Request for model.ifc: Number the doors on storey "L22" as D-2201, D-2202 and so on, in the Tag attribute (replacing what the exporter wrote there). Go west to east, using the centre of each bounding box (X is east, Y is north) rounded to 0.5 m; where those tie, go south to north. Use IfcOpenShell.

First a look at what the model holds.

```python
import ifcopenshell
import ifcopenshell.util.element
import ifcopenshell.util.placement

model = ifcopenshell.open("model.ifc")
print(model.schema)
storey = next(s for s in model.by_type("IfcBuildingStorey") if s.Name == "L22")
doors = [e for e in ifcopenshell.util.element.get_decomposition(storey) if e.is_a("IfcDoor")]
for e in sorted(doors, key=lambda e: e.id()):
    origin = ifcopenshell.util.placement.get_local_placement(e.ObjectPlacement)[:3, 3]
    print(e.id(), e.Tag, e.Name, origin.round(2) + 0.0, sep=" | ")
```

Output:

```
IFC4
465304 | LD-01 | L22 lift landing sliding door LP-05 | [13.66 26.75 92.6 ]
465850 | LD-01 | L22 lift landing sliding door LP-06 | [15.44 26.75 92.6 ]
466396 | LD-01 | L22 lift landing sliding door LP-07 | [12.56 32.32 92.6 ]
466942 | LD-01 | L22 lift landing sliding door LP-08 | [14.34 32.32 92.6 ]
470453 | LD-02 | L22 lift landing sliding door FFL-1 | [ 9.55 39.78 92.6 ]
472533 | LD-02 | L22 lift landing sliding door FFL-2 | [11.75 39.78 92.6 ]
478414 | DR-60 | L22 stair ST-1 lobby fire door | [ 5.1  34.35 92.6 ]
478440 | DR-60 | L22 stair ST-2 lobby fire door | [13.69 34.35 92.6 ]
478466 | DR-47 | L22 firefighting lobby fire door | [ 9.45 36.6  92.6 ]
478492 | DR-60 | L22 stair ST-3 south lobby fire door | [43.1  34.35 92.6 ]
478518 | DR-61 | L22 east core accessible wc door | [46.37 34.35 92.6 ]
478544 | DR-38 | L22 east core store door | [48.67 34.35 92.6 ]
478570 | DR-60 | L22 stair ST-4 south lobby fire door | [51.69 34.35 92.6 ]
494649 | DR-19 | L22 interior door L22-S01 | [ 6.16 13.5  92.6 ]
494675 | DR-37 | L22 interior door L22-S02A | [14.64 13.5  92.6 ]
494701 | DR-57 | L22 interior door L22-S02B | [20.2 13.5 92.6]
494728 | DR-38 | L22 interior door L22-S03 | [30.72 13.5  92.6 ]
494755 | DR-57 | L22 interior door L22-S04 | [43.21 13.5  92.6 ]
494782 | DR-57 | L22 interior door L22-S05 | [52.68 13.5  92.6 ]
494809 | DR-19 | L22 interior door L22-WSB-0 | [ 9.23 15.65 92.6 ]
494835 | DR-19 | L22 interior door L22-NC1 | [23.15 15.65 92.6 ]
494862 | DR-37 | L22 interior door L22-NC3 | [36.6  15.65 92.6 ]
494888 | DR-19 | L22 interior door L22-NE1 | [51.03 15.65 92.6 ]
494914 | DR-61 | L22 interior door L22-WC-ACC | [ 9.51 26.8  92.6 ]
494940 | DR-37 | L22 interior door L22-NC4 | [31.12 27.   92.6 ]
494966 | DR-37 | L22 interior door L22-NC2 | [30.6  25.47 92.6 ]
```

```python
import ifcopenshell
import ifcopenshell.geom
import ifcopenshell.util.element
import ifcopenshell.util.shape

model = ifcopenshell.open("model.ifc")
settings = ifcopenshell.geom.settings()
settings.set("use-world-coords", True)


def centre(element):
    shape = ifcopenshell.geom.create_shape(settings, element)
    return ifcopenshell.util.shape.get_bbox_centroid(shape.geometry)


storey = next(s for s in model.by_type("IfcBuildingStorey") if s.Name == "L22")
doors = [e for e in ifcopenshell.util.element.get_decomposition(storey) if e.is_a("IfcDoor")]

# Insertion points can sit at a corner or the storey origin, so sort by the geometry (in metres).
centres = {e: centre(e) for e in doors}
doors.sort(key=lambda e: (round(centres[e][0] / 0.5), centres[e][1]))

for i, e in enumerate(doors, start=1):
    number = f"D-22{i:02d}"
    e.Tag = number
    print(e.id(), number)

model.write("model_rev.ifc")
```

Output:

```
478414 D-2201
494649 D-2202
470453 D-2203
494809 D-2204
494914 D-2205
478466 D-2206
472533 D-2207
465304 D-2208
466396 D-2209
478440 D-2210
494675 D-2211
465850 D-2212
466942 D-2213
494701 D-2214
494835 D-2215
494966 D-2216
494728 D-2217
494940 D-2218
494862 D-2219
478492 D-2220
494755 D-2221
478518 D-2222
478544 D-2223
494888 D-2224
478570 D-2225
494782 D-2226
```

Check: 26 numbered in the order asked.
